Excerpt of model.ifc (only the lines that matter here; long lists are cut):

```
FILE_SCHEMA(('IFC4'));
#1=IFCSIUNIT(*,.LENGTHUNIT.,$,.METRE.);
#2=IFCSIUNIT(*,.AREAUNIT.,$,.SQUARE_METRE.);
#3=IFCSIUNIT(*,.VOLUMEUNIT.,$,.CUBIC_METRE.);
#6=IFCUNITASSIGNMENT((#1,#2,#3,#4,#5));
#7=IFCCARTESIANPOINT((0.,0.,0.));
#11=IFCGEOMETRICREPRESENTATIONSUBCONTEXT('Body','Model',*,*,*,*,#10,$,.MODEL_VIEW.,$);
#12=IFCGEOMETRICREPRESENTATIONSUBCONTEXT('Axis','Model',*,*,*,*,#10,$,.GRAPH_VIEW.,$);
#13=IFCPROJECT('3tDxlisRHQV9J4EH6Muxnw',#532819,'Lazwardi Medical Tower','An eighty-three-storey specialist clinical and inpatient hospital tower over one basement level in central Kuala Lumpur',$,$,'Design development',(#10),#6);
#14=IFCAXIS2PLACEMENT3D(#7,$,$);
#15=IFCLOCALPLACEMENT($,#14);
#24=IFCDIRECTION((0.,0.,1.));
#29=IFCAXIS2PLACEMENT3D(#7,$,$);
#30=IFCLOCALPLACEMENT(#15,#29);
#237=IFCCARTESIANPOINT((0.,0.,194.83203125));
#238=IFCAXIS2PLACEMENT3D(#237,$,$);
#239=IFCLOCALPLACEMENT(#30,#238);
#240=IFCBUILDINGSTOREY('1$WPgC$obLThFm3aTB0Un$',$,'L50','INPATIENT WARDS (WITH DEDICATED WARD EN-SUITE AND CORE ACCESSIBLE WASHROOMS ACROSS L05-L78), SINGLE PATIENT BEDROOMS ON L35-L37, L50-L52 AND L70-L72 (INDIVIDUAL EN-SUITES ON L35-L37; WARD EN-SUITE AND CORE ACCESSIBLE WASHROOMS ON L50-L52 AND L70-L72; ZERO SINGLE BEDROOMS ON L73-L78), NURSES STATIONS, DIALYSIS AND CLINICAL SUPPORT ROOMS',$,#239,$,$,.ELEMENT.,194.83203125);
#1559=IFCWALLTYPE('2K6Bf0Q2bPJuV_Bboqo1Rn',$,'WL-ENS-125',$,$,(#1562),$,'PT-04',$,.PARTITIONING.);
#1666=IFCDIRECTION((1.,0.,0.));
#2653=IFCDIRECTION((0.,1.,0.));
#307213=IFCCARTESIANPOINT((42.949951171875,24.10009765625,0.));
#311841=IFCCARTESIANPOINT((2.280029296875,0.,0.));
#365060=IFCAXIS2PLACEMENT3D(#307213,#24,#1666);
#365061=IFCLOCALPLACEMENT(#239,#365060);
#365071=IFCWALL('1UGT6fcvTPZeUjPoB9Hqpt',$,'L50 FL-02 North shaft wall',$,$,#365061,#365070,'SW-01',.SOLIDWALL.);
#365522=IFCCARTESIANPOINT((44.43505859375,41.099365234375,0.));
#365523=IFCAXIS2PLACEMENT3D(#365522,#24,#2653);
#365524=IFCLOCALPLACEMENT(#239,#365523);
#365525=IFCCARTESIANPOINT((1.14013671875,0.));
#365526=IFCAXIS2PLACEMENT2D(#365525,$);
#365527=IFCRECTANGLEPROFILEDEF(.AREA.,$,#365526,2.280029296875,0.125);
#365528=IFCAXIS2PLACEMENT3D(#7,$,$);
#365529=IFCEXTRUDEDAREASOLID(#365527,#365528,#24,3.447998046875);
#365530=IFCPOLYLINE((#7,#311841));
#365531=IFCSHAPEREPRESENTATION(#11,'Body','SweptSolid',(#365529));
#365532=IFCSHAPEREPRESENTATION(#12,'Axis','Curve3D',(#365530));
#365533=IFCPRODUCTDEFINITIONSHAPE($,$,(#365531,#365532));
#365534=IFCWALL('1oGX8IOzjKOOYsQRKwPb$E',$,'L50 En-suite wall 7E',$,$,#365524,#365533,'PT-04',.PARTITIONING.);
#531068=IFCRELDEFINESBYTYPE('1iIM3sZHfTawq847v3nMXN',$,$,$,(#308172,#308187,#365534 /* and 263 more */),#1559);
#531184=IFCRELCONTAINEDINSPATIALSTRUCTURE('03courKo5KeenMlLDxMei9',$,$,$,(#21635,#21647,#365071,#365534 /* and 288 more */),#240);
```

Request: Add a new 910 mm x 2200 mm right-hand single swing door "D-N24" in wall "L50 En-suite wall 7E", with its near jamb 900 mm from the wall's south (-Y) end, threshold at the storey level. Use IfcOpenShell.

```python
import numpy as np
import ifcopenshell
import ifcopenshell.api.feature
import ifcopenshell.api.geometry
import ifcopenshell.api.root
import ifcopenshell.api.spatial
import ifcopenshell.geom
import ifcopenshell.util.element
import ifcopenshell.util.placement
import ifcopenshell.util.representation
import ifcopenshell.util.shape
import ifcopenshell.util.unit

model = ifcopenshell.open("model.ifc")
unit_scale = ifcopenshell.util.unit.calculate_unit_scale(model)
settings = ifcopenshell.geom.settings()


def volume(element):
    """Net volume in cubic metres, openings subtracted."""
    shape = ifcopenshell.geom.create_shape(settings, element)
    return ifcopenshell.util.shape.get_volume(shape.geometry)


wall = model.by_id(365534)
storey = ifcopenshell.util.element.get_container(wall, ifc_class="IfcBuildingStorey")
context = ifcopenshell.util.representation.get_context(model, "Model", "Body", "MODEL_VIEW")
before = volume(wall)

width, height, from_end, sill = 0.91, 2.2, 0.9, 0.0  # metres

# The wall runs along its own X axis, and the end named is its -X end.
wall_shape = ifcopenshell.geom.create_shape(settings, wall)
x, y, z = ifcopenshell.util.shape.get_vertices(wall_shape.geometry).T
start = x.min() + from_end
face, thickness = float(y.min()), float(y.max() - y.min())
wall_matrix = ifcopenshell.util.placement.get_local_placement(wall.ObjectPlacement)
level = ifcopenshell.util.placement.get_local_placement(storey.ObjectPlacement)[2, 3]


def in_wall(x, y):
    """Placement at x, y metres in the wall's axes, at sill height."""
    matrix = wall_matrix.copy()
    matrix[:, 3] = wall_matrix @ np.array([x / unit_scale, y / unit_scale, 0.0, 1.0])
    matrix[2, 3] = level + sill / unit_scale
    return matrix


# Opening: a box that overshoots both wall faces by 50 mm.
opening = ifcopenshell.api.root.create_entity(model, ifc_class="IfcOpeningElement", predefined_type="OPENING")
box = ifcopenshell.api.geometry.add_wall_representation(
    model, context=context, length=width, height=height, thickness=thickness + 0.1
)
ifcopenshell.api.geometry.assign_representation(model, product=opening, representation=box)
ifcopenshell.api.geometry.edit_object_placement(model, product=opening, matrix=in_wall(start, face - 0.05), is_si=False)
ifcopenshell.api.feature.add_feature(model, feature=opening, element=wall)

door = ifcopenshell.api.root.create_entity(model, ifc_class="IfcDoor", name="D-N24", predefined_type="DOOR")
door.OverallWidth, door.OverallHeight = width / unit_scale, height / unit_scale
door.OperationType = "SINGLE_SWING_RIGHT"
body = ifcopenshell.api.geometry.add_door_representation(
    model,
    context=context,
    overall_width=door.OverallWidth,
    overall_height=door.OverallHeight,
    operation_type="SINGLE_SWING_RIGHT",
    lining_properties={"LiningDepth": thickness / unit_scale, "ThresholdDepth": thickness / unit_scale},
)
ifcopenshell.api.geometry.assign_representation(model, product=door, representation=body)
ifcopenshell.api.spatial.assign_container(model, products=[door], relating_structure=storey)
ifcopenshell.api.feature.add_filling(model, opening=opening, element=door)

# The lining spans the wall, so the door starts at the wall face.
ifcopenshell.api.geometry.edit_object_placement(model, product=door, matrix=in_wall(start, face), is_si=False)

after = volume(wall)

print(f"wall volume {before:.3f} -> {after:.3f} m3")

model.write("model_rev.ifc")
```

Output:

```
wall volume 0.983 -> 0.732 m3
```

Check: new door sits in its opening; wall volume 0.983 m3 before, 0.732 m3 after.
